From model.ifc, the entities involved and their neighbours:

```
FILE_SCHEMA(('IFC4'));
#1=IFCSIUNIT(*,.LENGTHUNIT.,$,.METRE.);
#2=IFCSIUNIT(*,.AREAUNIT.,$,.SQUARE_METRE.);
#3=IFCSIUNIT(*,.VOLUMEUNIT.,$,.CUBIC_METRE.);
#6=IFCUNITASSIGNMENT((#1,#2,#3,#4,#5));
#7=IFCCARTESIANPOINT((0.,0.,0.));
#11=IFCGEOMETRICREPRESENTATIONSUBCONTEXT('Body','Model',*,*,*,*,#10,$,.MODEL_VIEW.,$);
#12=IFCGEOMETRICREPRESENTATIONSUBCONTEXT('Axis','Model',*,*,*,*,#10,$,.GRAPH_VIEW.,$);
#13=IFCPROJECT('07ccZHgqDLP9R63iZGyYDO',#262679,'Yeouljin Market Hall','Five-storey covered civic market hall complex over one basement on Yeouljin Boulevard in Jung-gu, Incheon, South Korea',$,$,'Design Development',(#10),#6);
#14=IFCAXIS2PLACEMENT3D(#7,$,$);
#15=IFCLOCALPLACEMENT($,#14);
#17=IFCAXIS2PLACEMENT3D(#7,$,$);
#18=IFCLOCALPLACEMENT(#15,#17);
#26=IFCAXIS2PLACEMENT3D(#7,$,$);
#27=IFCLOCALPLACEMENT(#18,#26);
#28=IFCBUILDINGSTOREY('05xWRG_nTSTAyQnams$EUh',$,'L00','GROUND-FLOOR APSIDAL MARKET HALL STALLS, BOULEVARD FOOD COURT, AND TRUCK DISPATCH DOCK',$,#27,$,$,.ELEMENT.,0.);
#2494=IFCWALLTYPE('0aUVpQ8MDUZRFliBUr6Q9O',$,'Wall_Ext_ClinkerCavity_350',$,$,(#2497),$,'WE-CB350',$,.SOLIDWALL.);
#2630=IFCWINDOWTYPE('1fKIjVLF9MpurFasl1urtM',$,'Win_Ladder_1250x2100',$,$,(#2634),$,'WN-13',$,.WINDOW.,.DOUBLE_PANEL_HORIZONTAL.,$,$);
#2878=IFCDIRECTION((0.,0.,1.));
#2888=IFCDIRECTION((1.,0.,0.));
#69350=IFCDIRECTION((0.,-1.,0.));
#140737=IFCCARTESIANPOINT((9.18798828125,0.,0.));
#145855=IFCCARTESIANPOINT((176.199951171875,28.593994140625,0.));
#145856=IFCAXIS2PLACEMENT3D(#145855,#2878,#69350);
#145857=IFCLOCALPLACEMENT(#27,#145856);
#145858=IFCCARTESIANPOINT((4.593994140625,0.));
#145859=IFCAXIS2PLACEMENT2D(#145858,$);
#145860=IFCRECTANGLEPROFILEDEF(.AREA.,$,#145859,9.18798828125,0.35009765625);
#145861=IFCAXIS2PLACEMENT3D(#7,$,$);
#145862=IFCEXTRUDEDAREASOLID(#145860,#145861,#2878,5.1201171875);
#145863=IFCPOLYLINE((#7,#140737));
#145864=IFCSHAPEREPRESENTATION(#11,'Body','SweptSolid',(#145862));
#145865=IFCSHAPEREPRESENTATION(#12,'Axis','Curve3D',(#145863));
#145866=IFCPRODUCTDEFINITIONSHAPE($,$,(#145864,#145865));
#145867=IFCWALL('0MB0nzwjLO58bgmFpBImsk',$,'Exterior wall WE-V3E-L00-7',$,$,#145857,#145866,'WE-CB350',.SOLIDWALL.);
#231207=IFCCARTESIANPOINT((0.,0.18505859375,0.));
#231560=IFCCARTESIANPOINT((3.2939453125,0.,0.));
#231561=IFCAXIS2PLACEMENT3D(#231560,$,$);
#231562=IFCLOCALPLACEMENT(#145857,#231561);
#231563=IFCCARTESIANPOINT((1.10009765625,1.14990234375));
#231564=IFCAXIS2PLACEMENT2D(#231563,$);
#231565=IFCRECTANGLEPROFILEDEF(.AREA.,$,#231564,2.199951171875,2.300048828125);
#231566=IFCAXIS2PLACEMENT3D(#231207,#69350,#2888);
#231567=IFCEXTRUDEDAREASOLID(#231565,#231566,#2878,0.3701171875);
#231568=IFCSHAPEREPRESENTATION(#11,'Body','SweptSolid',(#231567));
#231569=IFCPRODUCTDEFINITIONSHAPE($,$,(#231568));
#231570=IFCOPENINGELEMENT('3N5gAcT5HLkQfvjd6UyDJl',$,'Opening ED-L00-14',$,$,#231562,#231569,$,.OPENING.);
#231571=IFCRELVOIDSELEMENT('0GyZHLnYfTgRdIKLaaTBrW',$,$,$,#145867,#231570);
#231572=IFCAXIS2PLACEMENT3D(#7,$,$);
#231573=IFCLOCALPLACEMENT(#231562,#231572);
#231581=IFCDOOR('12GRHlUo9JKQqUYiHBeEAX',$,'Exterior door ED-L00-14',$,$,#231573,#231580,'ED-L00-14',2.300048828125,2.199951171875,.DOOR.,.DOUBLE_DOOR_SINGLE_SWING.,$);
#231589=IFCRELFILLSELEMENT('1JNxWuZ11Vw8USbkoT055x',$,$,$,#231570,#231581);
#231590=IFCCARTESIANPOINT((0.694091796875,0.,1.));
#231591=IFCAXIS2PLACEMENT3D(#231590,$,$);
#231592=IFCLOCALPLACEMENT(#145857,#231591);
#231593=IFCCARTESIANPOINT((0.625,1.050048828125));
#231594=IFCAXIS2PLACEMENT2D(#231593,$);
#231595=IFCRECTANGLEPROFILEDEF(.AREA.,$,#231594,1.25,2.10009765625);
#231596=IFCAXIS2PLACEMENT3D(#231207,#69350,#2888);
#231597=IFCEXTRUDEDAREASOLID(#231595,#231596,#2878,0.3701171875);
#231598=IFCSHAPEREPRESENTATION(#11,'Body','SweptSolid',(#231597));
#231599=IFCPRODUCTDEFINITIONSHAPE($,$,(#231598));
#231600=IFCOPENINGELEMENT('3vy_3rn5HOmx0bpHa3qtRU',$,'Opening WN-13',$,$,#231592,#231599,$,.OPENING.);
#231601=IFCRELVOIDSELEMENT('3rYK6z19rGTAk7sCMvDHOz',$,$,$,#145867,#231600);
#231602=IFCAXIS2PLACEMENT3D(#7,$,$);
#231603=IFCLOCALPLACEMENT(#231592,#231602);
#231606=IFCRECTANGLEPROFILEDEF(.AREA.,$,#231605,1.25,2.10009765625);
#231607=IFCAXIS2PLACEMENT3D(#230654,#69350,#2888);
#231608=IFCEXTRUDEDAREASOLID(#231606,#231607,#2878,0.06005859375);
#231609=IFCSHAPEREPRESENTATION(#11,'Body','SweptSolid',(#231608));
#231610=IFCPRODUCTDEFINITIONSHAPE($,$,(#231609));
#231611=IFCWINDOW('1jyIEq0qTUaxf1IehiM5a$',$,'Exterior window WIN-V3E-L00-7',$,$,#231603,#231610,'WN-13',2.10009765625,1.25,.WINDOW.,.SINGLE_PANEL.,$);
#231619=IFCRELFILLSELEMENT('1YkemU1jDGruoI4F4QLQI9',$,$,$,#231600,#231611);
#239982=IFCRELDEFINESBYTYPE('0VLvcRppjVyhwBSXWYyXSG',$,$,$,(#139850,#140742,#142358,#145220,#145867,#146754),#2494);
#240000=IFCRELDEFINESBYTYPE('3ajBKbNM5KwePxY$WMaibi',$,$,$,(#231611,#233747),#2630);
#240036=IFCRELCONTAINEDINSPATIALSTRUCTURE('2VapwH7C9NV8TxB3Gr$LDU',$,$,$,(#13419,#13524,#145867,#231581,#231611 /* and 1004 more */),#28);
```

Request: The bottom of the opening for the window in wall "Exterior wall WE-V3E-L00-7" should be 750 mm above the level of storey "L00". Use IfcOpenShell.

```python
import numpy as np
import ifcopenshell
import ifcopenshell.api.geometry
import ifcopenshell.geom
import ifcopenshell.util.element
import ifcopenshell.util.placement
import ifcopenshell.util.shape
import ifcopenshell.util.unit

model = ifcopenshell.open("model.ifc")
unit_scale = ifcopenshell.util.unit.calculate_unit_scale(model)

window = model.by_id(231611)
opening = window.FillsVoids[0].RelatingOpeningElement
storey = ifcopenshell.util.element.get_container(window, ifc_class="IfcBuildingStorey")
level = ifcopenshell.util.placement.get_local_placement(storey.ObjectPlacement)[2, 3]

# The opening's origin need not be at the sill, so measure its lowest point.
shape = ifcopenshell.geom.create_shape(ifcopenshell.geom.settings(), opening)
bottom = ifcopenshell.util.shape.get_shape_bottom_elevation(shape, shape.geometry) / unit_scale
dz = level + 0.75 - bottom

shift = np.array([0.0, 0.0, dz])
# The window is placed relative to its opening, so it follows when the opening moves.
matrix = ifcopenshell.util.placement.get_local_placement(opening.ObjectPlacement)
matrix[:3, 3] += shift
ifcopenshell.api.geometry.edit_object_placement(
    model, product=opening, matrix=matrix, is_si=False, should_transform_children=True
)

print(f"moved by {dz * unit_scale:+.3f} m")

model.write("model-out.ifc")
```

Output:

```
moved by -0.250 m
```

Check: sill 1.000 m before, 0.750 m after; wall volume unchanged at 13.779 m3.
